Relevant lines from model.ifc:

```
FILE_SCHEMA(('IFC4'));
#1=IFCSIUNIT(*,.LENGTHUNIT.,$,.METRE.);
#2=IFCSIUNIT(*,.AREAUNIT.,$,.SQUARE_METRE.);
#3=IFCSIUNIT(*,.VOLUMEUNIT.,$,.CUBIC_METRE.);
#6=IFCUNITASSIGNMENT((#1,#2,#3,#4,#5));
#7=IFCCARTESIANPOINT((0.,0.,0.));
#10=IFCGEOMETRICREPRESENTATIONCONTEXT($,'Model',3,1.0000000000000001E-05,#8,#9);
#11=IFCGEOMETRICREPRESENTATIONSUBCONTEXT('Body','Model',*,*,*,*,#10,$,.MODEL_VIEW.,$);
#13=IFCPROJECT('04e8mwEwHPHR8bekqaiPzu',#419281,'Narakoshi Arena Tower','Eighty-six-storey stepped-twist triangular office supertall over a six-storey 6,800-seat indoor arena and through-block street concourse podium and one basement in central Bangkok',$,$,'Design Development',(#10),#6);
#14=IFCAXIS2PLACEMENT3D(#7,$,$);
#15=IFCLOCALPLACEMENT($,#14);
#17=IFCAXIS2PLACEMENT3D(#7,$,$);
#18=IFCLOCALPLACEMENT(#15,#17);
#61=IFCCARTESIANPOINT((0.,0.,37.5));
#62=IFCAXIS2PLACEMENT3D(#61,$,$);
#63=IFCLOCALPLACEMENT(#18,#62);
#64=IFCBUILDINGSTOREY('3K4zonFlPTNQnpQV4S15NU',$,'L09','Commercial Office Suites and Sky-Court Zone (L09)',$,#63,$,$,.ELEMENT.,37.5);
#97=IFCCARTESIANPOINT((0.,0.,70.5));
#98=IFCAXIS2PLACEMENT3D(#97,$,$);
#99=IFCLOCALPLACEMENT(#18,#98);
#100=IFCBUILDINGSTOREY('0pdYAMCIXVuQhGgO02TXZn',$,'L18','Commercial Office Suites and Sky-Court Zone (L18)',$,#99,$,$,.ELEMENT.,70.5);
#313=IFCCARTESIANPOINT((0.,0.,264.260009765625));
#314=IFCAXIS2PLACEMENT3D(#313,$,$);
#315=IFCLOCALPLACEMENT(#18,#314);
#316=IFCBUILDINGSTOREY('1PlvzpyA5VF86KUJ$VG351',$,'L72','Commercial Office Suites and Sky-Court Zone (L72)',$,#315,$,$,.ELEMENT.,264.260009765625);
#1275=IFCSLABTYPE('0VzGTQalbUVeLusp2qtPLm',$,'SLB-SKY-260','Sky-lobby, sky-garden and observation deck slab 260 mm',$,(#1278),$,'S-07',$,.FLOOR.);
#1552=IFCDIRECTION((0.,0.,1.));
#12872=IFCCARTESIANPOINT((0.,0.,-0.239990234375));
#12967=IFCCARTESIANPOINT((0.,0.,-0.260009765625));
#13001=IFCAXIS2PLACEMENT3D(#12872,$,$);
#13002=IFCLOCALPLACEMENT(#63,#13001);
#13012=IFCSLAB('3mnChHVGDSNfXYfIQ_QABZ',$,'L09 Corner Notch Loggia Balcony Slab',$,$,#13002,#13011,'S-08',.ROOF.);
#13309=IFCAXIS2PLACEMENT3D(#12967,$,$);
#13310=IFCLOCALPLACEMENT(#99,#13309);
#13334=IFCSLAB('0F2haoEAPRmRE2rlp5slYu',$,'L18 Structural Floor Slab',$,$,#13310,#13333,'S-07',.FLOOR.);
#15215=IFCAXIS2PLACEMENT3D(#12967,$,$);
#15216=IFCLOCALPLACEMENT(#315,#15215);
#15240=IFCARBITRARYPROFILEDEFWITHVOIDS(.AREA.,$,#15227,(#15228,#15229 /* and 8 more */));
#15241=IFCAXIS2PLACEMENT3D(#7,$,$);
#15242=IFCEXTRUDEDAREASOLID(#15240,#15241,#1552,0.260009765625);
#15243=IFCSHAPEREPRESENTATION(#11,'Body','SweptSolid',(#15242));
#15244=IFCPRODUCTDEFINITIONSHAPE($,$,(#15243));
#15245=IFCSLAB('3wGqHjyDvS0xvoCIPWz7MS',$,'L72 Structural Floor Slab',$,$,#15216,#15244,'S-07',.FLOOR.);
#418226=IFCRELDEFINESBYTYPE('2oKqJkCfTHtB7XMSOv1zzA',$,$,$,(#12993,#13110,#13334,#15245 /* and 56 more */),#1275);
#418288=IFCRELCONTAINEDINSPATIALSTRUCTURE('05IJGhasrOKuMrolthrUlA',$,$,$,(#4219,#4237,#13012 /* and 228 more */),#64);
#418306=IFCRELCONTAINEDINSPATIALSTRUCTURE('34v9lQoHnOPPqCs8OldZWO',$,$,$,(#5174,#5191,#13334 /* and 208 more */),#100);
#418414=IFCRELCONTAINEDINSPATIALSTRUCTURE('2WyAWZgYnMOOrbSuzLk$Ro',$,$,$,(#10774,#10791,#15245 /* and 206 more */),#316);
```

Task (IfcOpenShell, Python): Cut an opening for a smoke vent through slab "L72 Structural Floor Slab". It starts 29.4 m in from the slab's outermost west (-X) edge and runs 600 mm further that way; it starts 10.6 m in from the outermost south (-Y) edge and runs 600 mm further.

```python
import numpy as np
import ifcopenshell
import ifcopenshell.api.feature
import ifcopenshell.api.geometry
import ifcopenshell.api.root
import ifcopenshell.geom
import ifcopenshell.util.placement
import ifcopenshell.util.representation
import ifcopenshell.util.shape
import ifcopenshell.util.unit

model = ifcopenshell.open("model.ifc")
unit_scale = ifcopenshell.util.unit.calculate_unit_scale(model)
settings = ifcopenshell.geom.settings()


def volume(element):
    """Net volume in cubic metres, openings subtracted."""
    shape = ifcopenshell.geom.create_shape(settings, element)
    return ifcopenshell.util.shape.get_volume(shape.geometry)


slab = model.by_id(15245)
before = volume(slab)

# Extent in the slab's own axes, in metres. The edges named are its -X and -Y sides.
slab_shape = ifcopenshell.geom.create_shape(settings, slab)
vertices = ifcopenshell.util.shape.get_vertices(slab_shape.geometry)
x_min, y_min, bottom = vertices.min(axis=0)
top = vertices[:, 2].max()

opening = ifcopenshell.api.root.create_entity(model, ifc_class="IfcOpeningElement", name="Smoke vent opening", predefined_type="OPENING")
context = ifcopenshell.util.representation.get_context(model, "Model", "Body", "MODEL_VIEW")
width, depth = 0.6, 0.6
outline = [(0.0, 0.0), (width, 0.0), (width, depth), (0.0, depth), (0.0, 0.0)]
# Overshoot both faces by 50 mm so the cut is clean.
shape = ifcopenshell.api.geometry.add_slab_representation(
    model, context=context, depth=top - bottom + 0.1, polyline=outline
)
ifcopenshell.api.geometry.assign_representation(model, product=opening, representation=shape)

matrix = ifcopenshell.util.placement.get_local_placement(slab.ObjectPlacement)
matrix[:, 3] = matrix @ np.append(np.array([x_min + 29.4, y_min + 10.6, bottom - 0.05]) / unit_scale, 1.0)
ifcopenshell.api.geometry.edit_object_placement(model, product=opening, matrix=matrix, is_si=False)
ifcopenshell.api.feature.add_feature(model, feature=opening, element=slab)

after = volume(slab)

print(f"slab volume {before:.3f} -> {after:.3f} m3")

model.write("model_updated.ifc")
```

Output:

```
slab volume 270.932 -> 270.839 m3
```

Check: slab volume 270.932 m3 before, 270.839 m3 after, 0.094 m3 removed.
